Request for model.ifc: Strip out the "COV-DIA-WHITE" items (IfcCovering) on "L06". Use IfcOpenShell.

First a look at what the model holds.

```python
import ifcopenshell
import ifcopenshell.util.element

model = ifcopenshell.open("model.ifc")
print(model.schema)
storey = next(s for s in model.by_type("IfcBuildingStorey") if s.Name == "L06")
coverings = [e for e in ifcopenshell.util.element.get_decomposition(storey) if e.is_a("IfcCovering")]
seen = {}
for e in coverings:
    element_type = ifcopenshell.util.element.get_type(e)
    name = element_type.Name if element_type not in (None, e) else None
    seen[name] = seen.get(name, 0) + 1
for name, count in sorted(seen.items(), key=str):
    print(count, "x", name)
```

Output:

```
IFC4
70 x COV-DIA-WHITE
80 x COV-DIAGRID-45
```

```python
import ifcopenshell
import ifcopenshell.api.root
import ifcopenshell.util.element

model = ifcopenshell.open("model.ifc")

storey = next(s for s in model.by_type("IfcBuildingStorey") if s.Name == "L06")
coverings = [e for e in ifcopenshell.util.element.get_decomposition(storey) if e.is_a("IfcCovering")]
targets = [e for e in coverings if (t := ifcopenshell.util.element.get_type(e)) not in (None, e) and t.Name == "COV-DIA-WHITE"]

for e in targets:
    ifcopenshell.api.root.remove_product(model, product=e)
print(len(targets), "removed")

model.write("model_updated.ifc")
```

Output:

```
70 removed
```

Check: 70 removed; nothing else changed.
